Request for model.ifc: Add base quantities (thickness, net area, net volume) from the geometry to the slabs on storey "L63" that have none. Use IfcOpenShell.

First a look at what the model holds.

```python
import ifcopenshell
import ifcopenshell.util.element
import ifcopenshell.util.unit

model = ifcopenshell.open("model.ifc")
print(model.schema)
for unit_type in ("LENGTHUNIT", "AREAUNIT", "VOLUMEUNIT"):
    print(unit_type, ifcopenshell.util.unit.calculate_unit_scale(model, unit_type))
storey = next(s for s in model.by_type("IfcBuildingStorey") if s.Name == "L63")
slabs = [e for e in ifcopenshell.util.element.get_decomposition(storey) if e.is_a("IfcSlab")]
for e in sorted(slabs, key=lambda e: e.id()):
    print(e.id(), e.is_a(), e.Name, list(ifcopenshell.util.element.get_psets(e, qtos_only=True)), sep=" | ")
```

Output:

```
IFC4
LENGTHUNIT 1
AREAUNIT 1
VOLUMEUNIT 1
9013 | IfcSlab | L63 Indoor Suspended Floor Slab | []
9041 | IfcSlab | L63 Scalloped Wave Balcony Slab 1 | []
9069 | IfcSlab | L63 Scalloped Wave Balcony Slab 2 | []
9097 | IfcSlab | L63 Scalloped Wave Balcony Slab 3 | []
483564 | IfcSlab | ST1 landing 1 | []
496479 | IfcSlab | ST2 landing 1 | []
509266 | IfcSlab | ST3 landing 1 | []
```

```python
import ifcopenshell
import ifcopenshell.api.pset
import ifcopenshell.geom
import ifcopenshell.util.element
import ifcopenshell.util.shape
import ifcopenshell.util.unit

model = ifcopenshell.open("model.ifc")
unit_scale = ifcopenshell.util.unit.calculate_unit_scale(model)
area_scale = ifcopenshell.util.unit.calculate_unit_scale(model, "AREAUNIT")
volume_scale = ifcopenshell.util.unit.calculate_unit_scale(model, "VOLUMEUNIT")
settings = ifcopenshell.geom.settings()

storey = next(s for s in model.by_type("IfcBuildingStorey") if s.Name == "L63")
slabs = [e for e in ifcopenshell.util.element.get_decomposition(storey) if e.is_a("IfcSlab")]

for e in sorted(slabs, key=lambda e: e.id()):
    if ifcopenshell.util.element.get_psets(e, qtos_only=True, should_inherit=False):
        continue
    # Geometry comes back in metres, in the element's own axes.
    shape = ifcopenshell.geom.create_shape(settings, e)
    values = {
        "Width": ifcopenshell.util.shape.get_z(shape.geometry) / unit_scale,
        "NetArea": ifcopenshell.util.shape.get_footprint_area(shape.geometry) / area_scale,
        "NetVolume": ifcopenshell.util.shape.get_volume(shape.geometry) / volume_scale,
    }
    qto = ifcopenshell.api.pset.add_qto(model, product=e, name="Qto_SlabBaseQuantities")
    ifcopenshell.api.pset.edit_qto(model, qto=qto, properties=values)
    print(e.id(), {k: round(v, 3) for k, v in values.items()})

model.write("model_edited.ifc")
```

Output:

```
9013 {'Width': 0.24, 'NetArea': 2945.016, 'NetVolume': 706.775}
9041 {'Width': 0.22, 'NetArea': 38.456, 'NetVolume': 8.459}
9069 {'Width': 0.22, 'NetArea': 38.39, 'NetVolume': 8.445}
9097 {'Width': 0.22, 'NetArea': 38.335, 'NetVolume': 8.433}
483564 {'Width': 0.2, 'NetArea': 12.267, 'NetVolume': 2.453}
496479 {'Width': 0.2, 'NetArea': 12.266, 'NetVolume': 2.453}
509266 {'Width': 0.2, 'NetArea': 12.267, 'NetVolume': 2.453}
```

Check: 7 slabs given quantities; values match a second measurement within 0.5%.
